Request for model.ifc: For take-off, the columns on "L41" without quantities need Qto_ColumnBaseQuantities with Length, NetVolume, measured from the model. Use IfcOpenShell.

First a look at what the model holds.

```python
import ifcopenshell
import ifcopenshell.util.element
import ifcopenshell.util.unit

model = ifcopenshell.open("model.ifc")
print(model.schema)
for unit_type in ("LENGTHUNIT", "AREAUNIT", "VOLUMEUNIT"):
    print(unit_type, ifcopenshell.util.unit.calculate_unit_scale(model, unit_type))
storey = next(s for s in model.by_type("IfcBuildingStorey") if s.Name == "L41")
columns = [e for e in ifcopenshell.util.element.get_decomposition(storey) if e.is_a("IfcColumn")]
for e in sorted(columns, key=lambda e: e.id()):
    print(e.id(), e.is_a(), e.Name, list(ifcopenshell.util.element.get_psets(e, qtos_only=True)), sep=" | ")
```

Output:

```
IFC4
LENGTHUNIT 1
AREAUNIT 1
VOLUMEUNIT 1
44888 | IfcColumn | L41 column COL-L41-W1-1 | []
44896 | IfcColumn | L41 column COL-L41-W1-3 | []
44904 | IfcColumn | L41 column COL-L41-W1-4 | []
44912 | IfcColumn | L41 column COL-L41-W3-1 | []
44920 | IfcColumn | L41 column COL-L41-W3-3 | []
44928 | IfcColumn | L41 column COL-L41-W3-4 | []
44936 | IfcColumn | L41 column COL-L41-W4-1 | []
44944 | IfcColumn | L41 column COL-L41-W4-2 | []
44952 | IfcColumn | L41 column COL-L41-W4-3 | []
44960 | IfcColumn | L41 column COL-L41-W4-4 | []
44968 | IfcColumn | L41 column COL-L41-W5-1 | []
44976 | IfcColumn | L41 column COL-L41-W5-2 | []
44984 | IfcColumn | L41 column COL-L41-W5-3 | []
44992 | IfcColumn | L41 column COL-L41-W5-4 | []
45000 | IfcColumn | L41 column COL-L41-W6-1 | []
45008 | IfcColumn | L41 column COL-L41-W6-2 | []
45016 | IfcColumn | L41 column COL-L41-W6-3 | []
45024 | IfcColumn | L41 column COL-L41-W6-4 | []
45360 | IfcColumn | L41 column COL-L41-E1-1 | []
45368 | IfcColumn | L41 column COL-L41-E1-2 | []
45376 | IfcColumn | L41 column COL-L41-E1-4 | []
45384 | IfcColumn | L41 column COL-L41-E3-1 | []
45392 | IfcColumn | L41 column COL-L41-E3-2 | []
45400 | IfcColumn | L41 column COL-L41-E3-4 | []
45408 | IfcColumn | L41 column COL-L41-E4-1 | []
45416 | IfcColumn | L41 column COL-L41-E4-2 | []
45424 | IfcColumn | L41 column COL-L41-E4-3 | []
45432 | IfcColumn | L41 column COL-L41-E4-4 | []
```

```python
import ifcopenshell
import ifcopenshell.api.pset
import ifcopenshell.geom
import ifcopenshell.util.element
import ifcopenshell.util.shape
import ifcopenshell.util.unit

model = ifcopenshell.open("model.ifc")
unit_scale = ifcopenshell.util.unit.calculate_unit_scale(model)
volume_scale = ifcopenshell.util.unit.calculate_unit_scale(model, "VOLUMEUNIT")
settings = ifcopenshell.geom.settings()

storey = next(s for s in model.by_type("IfcBuildingStorey") if s.Name == "L41")
columns = [e for e in ifcopenshell.util.element.get_decomposition(storey) if e.is_a("IfcColumn")]

for e in sorted(columns, key=lambda e: e.id()):
    if ifcopenshell.util.element.get_psets(e, qtos_only=True, should_inherit=False):
        continue
    # Geometry comes back in metres, in the element's own axes.
    shape = ifcopenshell.geom.create_shape(settings, e)
    values = {
        "Length": ifcopenshell.util.shape.get_z(shape.geometry) / unit_scale,
        "NetVolume": ifcopenshell.util.shape.get_volume(shape.geometry) / volume_scale,
    }
    qto = ifcopenshell.api.pset.add_qto(model, product=e, name="Qto_ColumnBaseQuantities")
    ifcopenshell.api.pset.edit_qto(model, qto=qto, properties=values)
    print(e.id(), {k: round(v, 3) for k, v in values.items()})

model.write("model_rev.ifc")
```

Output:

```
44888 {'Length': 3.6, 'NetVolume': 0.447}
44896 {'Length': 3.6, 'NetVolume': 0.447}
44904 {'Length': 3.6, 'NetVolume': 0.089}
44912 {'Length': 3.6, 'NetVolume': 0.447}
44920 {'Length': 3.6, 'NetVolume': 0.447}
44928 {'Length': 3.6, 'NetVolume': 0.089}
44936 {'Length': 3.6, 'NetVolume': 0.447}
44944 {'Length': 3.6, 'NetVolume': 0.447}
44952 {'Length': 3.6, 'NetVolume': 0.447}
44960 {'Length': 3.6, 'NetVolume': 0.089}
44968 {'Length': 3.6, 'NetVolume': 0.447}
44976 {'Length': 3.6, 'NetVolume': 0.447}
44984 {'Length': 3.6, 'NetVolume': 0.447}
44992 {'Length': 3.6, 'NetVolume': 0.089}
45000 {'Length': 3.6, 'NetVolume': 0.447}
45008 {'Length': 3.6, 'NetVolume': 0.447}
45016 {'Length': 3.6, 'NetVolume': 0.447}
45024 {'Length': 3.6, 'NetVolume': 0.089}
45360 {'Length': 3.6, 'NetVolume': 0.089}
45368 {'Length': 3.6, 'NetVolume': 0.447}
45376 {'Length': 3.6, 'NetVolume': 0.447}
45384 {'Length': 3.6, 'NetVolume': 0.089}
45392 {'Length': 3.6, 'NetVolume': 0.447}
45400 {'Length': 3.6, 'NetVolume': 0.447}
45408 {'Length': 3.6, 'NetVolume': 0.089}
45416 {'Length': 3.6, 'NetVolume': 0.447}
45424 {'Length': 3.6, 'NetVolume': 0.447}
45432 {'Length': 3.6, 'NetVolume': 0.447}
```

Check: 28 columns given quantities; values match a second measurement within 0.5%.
